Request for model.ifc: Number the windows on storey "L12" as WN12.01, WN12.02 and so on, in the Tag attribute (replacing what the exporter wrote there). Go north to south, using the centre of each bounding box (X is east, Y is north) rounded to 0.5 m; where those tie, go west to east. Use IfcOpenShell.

First a look at what the model holds.

```python
import ifcopenshell
import ifcopenshell.util.element
import ifcopenshell.util.placement

model = ifcopenshell.open("model.ifc")
print(model.schema)
storey = next(s for s in model.by_type("IfcBuildingStorey") if s.Name == "L12")
windows = [e for e in ifcopenshell.util.element.get_decomposition(storey) if e.is_a("IfcWindow")]
for e in sorted(windows, key=lambda e: e.id()):
    origin = ifcopenshell.util.placement.get_local_placement(e.ObjectPlacement)[:3, 3]
    print(e.id(), e.Tag, e.Name, origin.round(2) + 0.0, sep=" | ")
```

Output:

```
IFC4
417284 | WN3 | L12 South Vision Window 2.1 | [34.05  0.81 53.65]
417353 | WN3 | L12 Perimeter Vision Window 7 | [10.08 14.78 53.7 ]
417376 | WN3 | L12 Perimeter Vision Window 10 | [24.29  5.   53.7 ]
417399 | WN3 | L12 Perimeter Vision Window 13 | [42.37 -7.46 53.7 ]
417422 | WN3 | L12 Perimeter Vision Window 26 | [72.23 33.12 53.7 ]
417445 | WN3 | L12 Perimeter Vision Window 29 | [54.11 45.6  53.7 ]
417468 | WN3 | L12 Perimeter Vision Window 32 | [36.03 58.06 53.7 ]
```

```python
import ifcopenshell
import ifcopenshell.geom
import ifcopenshell.util.element
import ifcopenshell.util.shape

model = ifcopenshell.open("model.ifc")
settings = ifcopenshell.geom.settings()
settings.set("use-world-coords", True)


def centre(element):
    shape = ifcopenshell.geom.create_shape(settings, element)
    return ifcopenshell.util.shape.get_bbox_centroid(shape.geometry)


storey = next(s for s in model.by_type("IfcBuildingStorey") if s.Name == "L12")
windows = [e for e in ifcopenshell.util.element.get_decomposition(storey) if e.is_a("IfcWindow")]

# Insertion points can sit at a corner or the storey origin, so sort by the geometry (in metres).
centres = {e: centre(e) for e in windows}
windows.sort(key=lambda e: (-round(centres[e][1] / 0.5), centres[e][0]))

for i, e in enumerate(windows, start=1):
    number = f"WN12.{i:02d}"
    e.Tag = number
    print(e.id(), number)

model.write("model_updated.ifc")
```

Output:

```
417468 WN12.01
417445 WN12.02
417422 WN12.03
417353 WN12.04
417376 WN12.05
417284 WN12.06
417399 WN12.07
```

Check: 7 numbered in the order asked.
